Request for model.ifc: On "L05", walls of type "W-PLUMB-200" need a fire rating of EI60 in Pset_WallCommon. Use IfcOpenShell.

First a look at what the model holds.

```python
import ifcopenshell
import ifcopenshell.util.element

model = ifcopenshell.open("model.ifc")
print(model.schema)
storey = next(s for s in model.by_type("IfcBuildingStorey") if s.Name == "L05")
walls = [e for e in ifcopenshell.util.element.get_decomposition(storey) if e.is_a("IfcWall")]
seen = {}
for e in walls:
    element_type = ifcopenshell.util.element.get_type(e)
    key = (element_type.Name if element_type != e and element_type else None, ifcopenshell.util.element.get_pset(e, "Pset_WallCommon", "FireRating"))
    seen[key] = seen.get(key, 0) + 1
for (name, value), count in sorted(seen.items(), key=str):
    print(count, "x", name, "|", value)
```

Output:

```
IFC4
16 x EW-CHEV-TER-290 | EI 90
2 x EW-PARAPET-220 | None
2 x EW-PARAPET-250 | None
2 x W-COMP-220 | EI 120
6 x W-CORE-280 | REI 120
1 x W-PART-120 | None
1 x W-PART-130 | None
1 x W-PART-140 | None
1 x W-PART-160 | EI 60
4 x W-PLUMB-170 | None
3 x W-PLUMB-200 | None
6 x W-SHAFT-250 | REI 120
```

```python
import ifcopenshell
import ifcopenshell.api.pset
import ifcopenshell.util.element

model = ifcopenshell.open("model.ifc")

storey = next(s for s in model.by_type("IfcBuildingStorey") if s.Name == "L05")
walls = [e for e in ifcopenshell.util.element.get_decomposition(storey) if e.is_a("IfcWall")]

count = 0
for e in walls:
    element_type = ifcopenshell.util.element.get_type(e)
    if element_type in (None, e) or element_type.Name != "W-PLUMB-200":
        continue
    # add_pset returns the element's existing set when there is one.
    pset = ifcopenshell.api.pset.add_pset(model, product=e, name="Pset_WallCommon")
    ifcopenshell.api.pset.edit_pset(model, pset=pset, properties={"FireRating": "EI60"})
    count += 1

print(count, "walls updated")

model.write("model_v2.ifc")
```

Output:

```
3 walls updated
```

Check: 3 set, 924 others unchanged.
